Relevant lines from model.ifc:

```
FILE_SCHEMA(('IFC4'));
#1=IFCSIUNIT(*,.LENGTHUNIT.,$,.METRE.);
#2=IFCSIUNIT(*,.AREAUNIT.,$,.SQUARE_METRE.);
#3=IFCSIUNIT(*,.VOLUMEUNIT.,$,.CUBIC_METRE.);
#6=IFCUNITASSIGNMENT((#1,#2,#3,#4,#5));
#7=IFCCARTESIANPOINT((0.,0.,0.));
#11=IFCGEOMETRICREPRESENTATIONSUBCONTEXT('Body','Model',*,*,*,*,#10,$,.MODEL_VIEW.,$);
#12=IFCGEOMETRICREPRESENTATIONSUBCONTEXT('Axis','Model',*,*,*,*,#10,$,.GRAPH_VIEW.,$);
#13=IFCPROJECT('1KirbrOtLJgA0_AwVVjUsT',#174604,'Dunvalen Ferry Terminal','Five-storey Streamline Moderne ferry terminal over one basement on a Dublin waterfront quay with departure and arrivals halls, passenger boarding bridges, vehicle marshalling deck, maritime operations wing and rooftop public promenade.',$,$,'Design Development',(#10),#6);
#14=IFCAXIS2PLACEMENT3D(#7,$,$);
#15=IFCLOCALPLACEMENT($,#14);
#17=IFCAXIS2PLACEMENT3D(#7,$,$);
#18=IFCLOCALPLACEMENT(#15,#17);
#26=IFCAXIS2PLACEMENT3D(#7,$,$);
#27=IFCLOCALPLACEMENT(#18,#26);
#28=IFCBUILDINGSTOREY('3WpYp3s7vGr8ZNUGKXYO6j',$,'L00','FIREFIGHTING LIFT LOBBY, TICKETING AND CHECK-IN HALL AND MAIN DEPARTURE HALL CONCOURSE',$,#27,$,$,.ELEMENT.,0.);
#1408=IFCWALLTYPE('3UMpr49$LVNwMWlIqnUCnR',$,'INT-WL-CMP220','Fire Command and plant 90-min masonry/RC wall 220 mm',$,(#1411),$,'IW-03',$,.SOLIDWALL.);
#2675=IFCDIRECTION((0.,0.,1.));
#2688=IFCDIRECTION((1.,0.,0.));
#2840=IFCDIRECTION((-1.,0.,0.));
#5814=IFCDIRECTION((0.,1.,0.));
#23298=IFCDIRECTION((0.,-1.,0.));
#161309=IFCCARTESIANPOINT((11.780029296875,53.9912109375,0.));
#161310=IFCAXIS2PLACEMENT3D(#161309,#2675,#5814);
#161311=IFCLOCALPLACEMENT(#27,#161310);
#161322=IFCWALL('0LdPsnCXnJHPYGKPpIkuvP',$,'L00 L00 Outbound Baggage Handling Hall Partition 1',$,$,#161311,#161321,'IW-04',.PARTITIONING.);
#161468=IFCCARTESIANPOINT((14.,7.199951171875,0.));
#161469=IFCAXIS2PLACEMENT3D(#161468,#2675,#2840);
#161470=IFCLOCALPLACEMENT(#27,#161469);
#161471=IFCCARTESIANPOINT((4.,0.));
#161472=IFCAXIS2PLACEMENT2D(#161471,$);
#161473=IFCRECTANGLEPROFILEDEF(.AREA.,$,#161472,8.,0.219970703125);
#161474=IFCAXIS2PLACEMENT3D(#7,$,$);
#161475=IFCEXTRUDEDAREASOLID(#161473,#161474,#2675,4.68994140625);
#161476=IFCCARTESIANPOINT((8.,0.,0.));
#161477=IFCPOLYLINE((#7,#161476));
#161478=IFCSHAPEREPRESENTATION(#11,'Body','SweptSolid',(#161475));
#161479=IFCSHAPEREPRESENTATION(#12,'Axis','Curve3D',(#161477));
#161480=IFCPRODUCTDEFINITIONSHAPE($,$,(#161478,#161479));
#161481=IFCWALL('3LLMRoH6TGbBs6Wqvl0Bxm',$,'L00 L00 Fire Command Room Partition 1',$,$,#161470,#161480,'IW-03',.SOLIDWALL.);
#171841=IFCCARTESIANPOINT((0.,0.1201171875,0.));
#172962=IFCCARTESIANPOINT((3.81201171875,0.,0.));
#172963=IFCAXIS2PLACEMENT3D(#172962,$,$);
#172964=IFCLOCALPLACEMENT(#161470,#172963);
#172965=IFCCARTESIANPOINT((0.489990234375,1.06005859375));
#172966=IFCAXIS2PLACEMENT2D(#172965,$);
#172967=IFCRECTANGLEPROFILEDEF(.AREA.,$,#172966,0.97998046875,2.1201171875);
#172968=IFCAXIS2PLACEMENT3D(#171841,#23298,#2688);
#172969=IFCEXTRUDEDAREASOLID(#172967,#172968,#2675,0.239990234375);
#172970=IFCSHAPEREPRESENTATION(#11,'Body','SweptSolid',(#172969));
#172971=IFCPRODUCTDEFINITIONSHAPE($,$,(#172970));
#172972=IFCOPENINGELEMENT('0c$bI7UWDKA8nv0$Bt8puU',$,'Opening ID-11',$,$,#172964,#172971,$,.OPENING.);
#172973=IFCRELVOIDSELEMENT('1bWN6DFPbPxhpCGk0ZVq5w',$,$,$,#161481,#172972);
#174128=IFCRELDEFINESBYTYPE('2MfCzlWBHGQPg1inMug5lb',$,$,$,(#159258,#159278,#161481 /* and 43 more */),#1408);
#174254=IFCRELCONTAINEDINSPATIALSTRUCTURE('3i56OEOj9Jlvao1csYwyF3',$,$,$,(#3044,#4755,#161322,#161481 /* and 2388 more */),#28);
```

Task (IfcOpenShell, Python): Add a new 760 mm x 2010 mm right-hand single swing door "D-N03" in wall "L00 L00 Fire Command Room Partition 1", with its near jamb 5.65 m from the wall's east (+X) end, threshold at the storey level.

```python
import numpy as np
import ifcopenshell
import ifcopenshell.api.feature
import ifcopenshell.api.geometry
import ifcopenshell.api.root
import ifcopenshell.api.spatial
import ifcopenshell.geom
import ifcopenshell.util.element
import ifcopenshell.util.placement
import ifcopenshell.util.representation
import ifcopenshell.util.shape
import ifcopenshell.util.unit

model = ifcopenshell.open("model.ifc")
unit_scale = ifcopenshell.util.unit.calculate_unit_scale(model)
settings = ifcopenshell.geom.settings()


def volume(element):
    """Net volume in cubic metres, openings subtracted."""
    shape = ifcopenshell.geom.create_shape(settings, element)
    return ifcopenshell.util.shape.get_volume(shape.geometry)


wall = model.by_id(161481)
storey = ifcopenshell.util.element.get_container(wall, ifc_class="IfcBuildingStorey")
context = ifcopenshell.util.representation.get_context(model, "Model", "Body", "MODEL_VIEW")
before = volume(wall)

width, height, from_end, sill = 0.76, 2.01, 5.65, 0.0  # metres

# The wall runs along its own X axis, and the end named is its -X end.
wall_shape = ifcopenshell.geom.create_shape(settings, wall)
x, y, z = ifcopenshell.util.shape.get_vertices(wall_shape.geometry).T
start = x.min() + from_end
face, thickness = float(y.min()), float(y.max() - y.min())
wall_matrix = ifcopenshell.util.placement.get_local_placement(wall.ObjectPlacement)
level = ifcopenshell.util.placement.get_local_placement(storey.ObjectPlacement)[2, 3]


def in_wall(x, y):
    """Placement at x, y metres in the wall's axes, at sill height."""
    matrix = wall_matrix.copy()
    matrix[:, 3] = wall_matrix @ np.array([x / unit_scale, y / unit_scale, 0.0, 1.0])
    matrix[2, 3] = level + sill / unit_scale
    return matrix


# Opening: a box that overshoots both wall faces by 50 mm.
opening = ifcopenshell.api.root.create_entity(model, ifc_class="IfcOpeningElement", predefined_type="OPENING")
box = ifcopenshell.api.geometry.add_wall_representation(
    model, context=context, length=width, height=height, thickness=thickness + 0.1
)
ifcopenshell.api.geometry.assign_representation(model, product=opening, representation=box)
ifcopenshell.api.geometry.edit_object_placement(model, product=opening, matrix=in_wall(start, face - 0.05), is_si=False)
ifcopenshell.api.feature.add_feature(model, feature=opening, element=wall)

door = ifcopenshell.api.root.create_entity(model, ifc_class="IfcDoor", name="D-N03", predefined_type="DOOR")
door.OverallWidth, door.OverallHeight = width / unit_scale, height / unit_scale
door.OperationType = "SINGLE_SWING_RIGHT"
body = ifcopenshell.api.geometry.add_door_representation(
    model,
    context=context,
    overall_width=door.OverallWidth,
    overall_height=door.OverallHeight,
    operation_type="SINGLE_SWING_RIGHT",
    lining_properties={"LiningDepth": thickness / unit_scale, "ThresholdDepth": thickness / unit_scale},
)
ifcopenshell.api.geometry.assign_representation(model, product=door, representation=body)
ifcopenshell.api.spatial.assign_container(model, products=[door], relating_structure=storey)
ifcopenshell.api.feature.add_filling(model, opening=opening, element=door)

# The lining spans the wall, so the door starts at the wall face.
ifcopenshell.api.geometry.edit_object_placement(model, product=door, matrix=in_wall(start, face), is_si=False)

after = volume(wall)

print(f"wall volume {before:.3f} -> {after:.3f} m3")

model.write("model-out.ifc")
```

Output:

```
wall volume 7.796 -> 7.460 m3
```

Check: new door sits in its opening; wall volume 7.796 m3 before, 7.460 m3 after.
